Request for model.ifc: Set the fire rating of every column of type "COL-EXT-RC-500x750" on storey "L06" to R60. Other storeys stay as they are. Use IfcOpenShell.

First a look at what the model holds.

```python
import ifcopenshell
import ifcopenshell.util.element

model = ifcopenshell.open("model.ifc")
print(model.schema)
storey = next(s for s in model.by_type("IfcBuildingStorey") if s.Name == "L06")
columns = [e for e in ifcopenshell.util.element.get_decomposition(storey) if e.is_a("IfcColumn")]
seen = {}
for e in columns:
    element_type = ifcopenshell.util.element.get_type(e)
    key = (element_type.Name if element_type != e and element_type else None, ifcopenshell.util.element.get_pset(e, "Pset_ColumnCommon", "FireRating"))
    seen[key] = seen.get(key, 0) + 1
for (name, value), count in sorted(seen.items(), key=str):
    print(count, "x", name, "|", value)
```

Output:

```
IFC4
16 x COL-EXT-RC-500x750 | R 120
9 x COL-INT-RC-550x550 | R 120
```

```python
import ifcopenshell
import ifcopenshell.api.pset
import ifcopenshell.util.element

model = ifcopenshell.open("model.ifc")

storey = next(s for s in model.by_type("IfcBuildingStorey") if s.Name == "L06")
columns = [e for e in ifcopenshell.util.element.get_decomposition(storey) if e.is_a("IfcColumn")]

count = 0
for e in columns:
    element_type = ifcopenshell.util.element.get_type(e)
    if element_type in (None, e) or element_type.Name != "COL-EXT-RC-500x750":
        continue
    # add_pset returns the element's existing set when there is one.
    pset = ifcopenshell.api.pset.add_pset(model, product=e, name="Pset_ColumnCommon")
    ifcopenshell.api.pset.edit_pset(model, pset=pset, properties={"FireRating": "R60"})
    count += 1

print(count, "columns updated")

model.write("model_v2.ifc")
```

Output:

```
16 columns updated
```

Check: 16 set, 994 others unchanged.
